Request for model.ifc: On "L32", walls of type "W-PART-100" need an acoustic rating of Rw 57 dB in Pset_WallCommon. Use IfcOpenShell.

First a look at what the model holds.

```python
import ifcopenshell
import ifcopenshell.util.element

model = ifcopenshell.open("model.ifc")
print(model.schema)
storey = next(s for s in model.by_type("IfcBuildingStorey") if s.Name == "L32")
walls = [e for e in ifcopenshell.util.element.get_decomposition(storey) if e.is_a("IfcWall")]
seen = {}
for e in walls:
    element_type = ifcopenshell.util.element.get_type(e)
    key = (element_type.Name if element_type != e and element_type else None, ifcopenshell.util.element.get_pset(e, "Pset_WallCommon", "AcousticRating"))
    seen[key] = seen.get(key, 0) + 1
for (name, value), count in sorted(seen.items(), key=str):
    print(count, "x", name, "|", value)
```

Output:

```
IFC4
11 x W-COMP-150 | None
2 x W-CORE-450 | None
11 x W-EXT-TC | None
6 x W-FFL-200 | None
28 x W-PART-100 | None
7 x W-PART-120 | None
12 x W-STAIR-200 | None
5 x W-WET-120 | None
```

```python
import ifcopenshell
import ifcopenshell.api.pset
import ifcopenshell.util.element

model = ifcopenshell.open("model.ifc")

storey = next(s for s in model.by_type("IfcBuildingStorey") if s.Name == "L32")
walls = [e for e in ifcopenshell.util.element.get_decomposition(storey) if e.is_a("IfcWall")]

count = 0
for e in walls:
    element_type = ifcopenshell.util.element.get_type(e)
    if element_type in (None, e) or element_type.Name != "W-PART-100":
        continue
    found = ifcopenshell.util.element.get_pset(e, "Pset_WallCommon", should_inherit=False)
    if found:
        pset = model.by_id(found["id"])
        if len(ifcopenshell.util.element.get_elements_by_pset(pset)) > 1:
            pset = ifcopenshell.api.pset.unshare_pset(model, products=[e], pset=pset)[0]
    else:
        pset = ifcopenshell.api.pset.add_pset(model, product=e, name="Pset_WallCommon")
    ifcopenshell.api.pset.edit_pset(model, pset=pset, properties={"AcousticRating": "Rw 57 dB"})
    count += 1

print(count, "walls updated")

model.write("model_rev.ifc")
```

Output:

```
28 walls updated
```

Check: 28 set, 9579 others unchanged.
